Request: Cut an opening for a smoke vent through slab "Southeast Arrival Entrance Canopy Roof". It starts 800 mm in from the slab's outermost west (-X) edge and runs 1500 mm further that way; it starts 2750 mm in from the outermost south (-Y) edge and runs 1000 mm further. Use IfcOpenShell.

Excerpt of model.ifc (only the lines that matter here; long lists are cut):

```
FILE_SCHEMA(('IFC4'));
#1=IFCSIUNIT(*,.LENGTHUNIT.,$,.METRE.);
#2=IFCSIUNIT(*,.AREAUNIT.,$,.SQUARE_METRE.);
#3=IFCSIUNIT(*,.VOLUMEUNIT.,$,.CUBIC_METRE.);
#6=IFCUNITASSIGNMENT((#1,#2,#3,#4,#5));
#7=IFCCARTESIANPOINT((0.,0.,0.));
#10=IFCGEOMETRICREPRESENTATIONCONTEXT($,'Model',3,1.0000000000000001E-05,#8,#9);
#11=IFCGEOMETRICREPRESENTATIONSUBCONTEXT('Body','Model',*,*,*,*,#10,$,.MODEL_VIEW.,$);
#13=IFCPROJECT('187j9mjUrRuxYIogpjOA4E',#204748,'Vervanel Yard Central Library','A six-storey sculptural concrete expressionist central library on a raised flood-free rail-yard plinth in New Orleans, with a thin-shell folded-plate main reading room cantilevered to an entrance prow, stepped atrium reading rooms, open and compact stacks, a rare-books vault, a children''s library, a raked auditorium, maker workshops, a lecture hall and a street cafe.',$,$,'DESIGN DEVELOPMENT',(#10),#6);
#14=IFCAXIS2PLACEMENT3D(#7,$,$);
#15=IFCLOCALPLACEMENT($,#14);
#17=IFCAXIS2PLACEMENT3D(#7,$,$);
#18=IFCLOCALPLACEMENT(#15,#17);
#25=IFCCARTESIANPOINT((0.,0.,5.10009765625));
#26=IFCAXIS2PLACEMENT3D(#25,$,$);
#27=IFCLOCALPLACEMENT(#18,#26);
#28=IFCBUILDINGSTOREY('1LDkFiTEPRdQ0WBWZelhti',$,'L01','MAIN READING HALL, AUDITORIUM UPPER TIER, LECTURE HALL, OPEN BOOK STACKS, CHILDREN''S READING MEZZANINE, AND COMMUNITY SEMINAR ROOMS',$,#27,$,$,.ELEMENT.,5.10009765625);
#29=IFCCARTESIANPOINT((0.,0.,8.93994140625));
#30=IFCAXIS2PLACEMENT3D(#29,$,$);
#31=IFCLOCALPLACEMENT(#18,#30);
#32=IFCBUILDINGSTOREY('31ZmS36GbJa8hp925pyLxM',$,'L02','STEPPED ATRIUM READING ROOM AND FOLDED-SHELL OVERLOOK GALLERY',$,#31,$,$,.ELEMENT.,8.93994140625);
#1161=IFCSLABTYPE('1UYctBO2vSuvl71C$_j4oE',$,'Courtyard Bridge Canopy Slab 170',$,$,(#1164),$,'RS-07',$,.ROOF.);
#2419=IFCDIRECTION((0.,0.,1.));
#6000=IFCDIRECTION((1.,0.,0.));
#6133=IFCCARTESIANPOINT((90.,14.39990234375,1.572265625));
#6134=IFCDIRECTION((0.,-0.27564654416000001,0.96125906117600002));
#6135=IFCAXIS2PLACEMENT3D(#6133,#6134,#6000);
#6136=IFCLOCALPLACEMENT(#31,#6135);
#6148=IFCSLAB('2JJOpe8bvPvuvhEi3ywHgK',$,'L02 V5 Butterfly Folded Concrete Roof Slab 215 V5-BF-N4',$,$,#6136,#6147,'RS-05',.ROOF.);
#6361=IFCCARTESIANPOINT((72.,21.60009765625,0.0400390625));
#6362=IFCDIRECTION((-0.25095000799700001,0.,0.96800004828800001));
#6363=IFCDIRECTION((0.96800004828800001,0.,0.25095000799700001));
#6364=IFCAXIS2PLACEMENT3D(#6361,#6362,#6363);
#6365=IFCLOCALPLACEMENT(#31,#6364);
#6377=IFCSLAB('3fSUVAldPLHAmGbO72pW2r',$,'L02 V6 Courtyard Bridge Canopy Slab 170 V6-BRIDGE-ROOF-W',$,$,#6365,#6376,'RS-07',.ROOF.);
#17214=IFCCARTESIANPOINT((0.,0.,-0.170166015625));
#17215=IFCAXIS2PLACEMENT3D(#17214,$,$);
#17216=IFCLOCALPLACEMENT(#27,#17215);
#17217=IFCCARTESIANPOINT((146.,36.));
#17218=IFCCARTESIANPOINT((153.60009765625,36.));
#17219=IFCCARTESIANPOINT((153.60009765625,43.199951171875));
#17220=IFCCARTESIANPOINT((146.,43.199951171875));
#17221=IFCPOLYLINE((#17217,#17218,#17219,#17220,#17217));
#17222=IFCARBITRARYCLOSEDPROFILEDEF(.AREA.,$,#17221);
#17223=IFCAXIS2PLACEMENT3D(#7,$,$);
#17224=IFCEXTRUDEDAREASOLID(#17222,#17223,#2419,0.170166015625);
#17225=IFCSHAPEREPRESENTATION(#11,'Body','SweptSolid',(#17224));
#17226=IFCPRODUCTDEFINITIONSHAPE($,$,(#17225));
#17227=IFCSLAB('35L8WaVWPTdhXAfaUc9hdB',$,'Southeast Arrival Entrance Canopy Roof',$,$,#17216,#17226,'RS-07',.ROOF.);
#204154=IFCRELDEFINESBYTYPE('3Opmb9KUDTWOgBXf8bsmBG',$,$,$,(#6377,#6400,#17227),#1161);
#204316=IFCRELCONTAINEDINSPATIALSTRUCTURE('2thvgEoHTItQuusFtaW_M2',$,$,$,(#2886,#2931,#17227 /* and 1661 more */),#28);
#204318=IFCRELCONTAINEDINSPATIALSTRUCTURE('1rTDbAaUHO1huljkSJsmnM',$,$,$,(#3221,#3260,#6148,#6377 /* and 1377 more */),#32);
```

```python
import numpy as np
import ifcopenshell
import ifcopenshell.api.feature
import ifcopenshell.api.geometry
import ifcopenshell.api.root
import ifcopenshell.geom
import ifcopenshell.util.placement
import ifcopenshell.util.representation
import ifcopenshell.util.shape
import ifcopenshell.util.unit

model = ifcopenshell.open("model.ifc")
unit_scale = ifcopenshell.util.unit.calculate_unit_scale(model)
settings = ifcopenshell.geom.settings()


def volume(element):
    """Net volume in cubic metres, openings subtracted."""
    shape = ifcopenshell.geom.create_shape(settings, element)
    return ifcopenshell.util.shape.get_volume(shape.geometry)


slab = model.by_guid("35L8WaVWPTdhXAfaUc9hdB")
before = volume(slab)

# Extent in the slab's own axes, in metres. The edges named are its -X and -Y sides.
slab_shape = ifcopenshell.geom.create_shape(settings, slab)
vertices = ifcopenshell.util.shape.get_vertices(slab_shape.geometry)
x_min, y_min, bottom = vertices.min(axis=0)
top = vertices[:, 2].max()

opening = ifcopenshell.api.root.create_entity(model, ifc_class="IfcOpeningElement", name="Smoke vent opening", predefined_type="OPENING")
context = ifcopenshell.util.representation.get_context(model, "Model", "Body", "MODEL_VIEW")
width, depth = 1.5, 1
outline = [(0.0, 0.0), (width, 0.0), (width, depth), (0.0, depth), (0.0, 0.0)]
# Overshoot both faces by 50 mm so the cut is clean.
shape = ifcopenshell.api.geometry.add_slab_representation(
    model, context=context, depth=top - bottom + 0.1, polyline=outline
)
ifcopenshell.api.geometry.assign_representation(model, product=opening, representation=shape)

matrix = ifcopenshell.util.placement.get_local_placement(slab.ObjectPlacement)
matrix[:, 3] = matrix @ np.append(np.array([x_min + 0.8, y_min + 2.75, bottom - 0.05]) / unit_scale, 1.0)
ifcopenshell.api.geometry.edit_object_placement(model, product=opening, matrix=matrix, is_si=False)
ifcopenshell.api.feature.add_feature(model, feature=opening, element=slab)

after = volume(slab)

print(f"slab volume {before:.3f} -> {after:.3f} m3")

model.write("model-out.ifc")
```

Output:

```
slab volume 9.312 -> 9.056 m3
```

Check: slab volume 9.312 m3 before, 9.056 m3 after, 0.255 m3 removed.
